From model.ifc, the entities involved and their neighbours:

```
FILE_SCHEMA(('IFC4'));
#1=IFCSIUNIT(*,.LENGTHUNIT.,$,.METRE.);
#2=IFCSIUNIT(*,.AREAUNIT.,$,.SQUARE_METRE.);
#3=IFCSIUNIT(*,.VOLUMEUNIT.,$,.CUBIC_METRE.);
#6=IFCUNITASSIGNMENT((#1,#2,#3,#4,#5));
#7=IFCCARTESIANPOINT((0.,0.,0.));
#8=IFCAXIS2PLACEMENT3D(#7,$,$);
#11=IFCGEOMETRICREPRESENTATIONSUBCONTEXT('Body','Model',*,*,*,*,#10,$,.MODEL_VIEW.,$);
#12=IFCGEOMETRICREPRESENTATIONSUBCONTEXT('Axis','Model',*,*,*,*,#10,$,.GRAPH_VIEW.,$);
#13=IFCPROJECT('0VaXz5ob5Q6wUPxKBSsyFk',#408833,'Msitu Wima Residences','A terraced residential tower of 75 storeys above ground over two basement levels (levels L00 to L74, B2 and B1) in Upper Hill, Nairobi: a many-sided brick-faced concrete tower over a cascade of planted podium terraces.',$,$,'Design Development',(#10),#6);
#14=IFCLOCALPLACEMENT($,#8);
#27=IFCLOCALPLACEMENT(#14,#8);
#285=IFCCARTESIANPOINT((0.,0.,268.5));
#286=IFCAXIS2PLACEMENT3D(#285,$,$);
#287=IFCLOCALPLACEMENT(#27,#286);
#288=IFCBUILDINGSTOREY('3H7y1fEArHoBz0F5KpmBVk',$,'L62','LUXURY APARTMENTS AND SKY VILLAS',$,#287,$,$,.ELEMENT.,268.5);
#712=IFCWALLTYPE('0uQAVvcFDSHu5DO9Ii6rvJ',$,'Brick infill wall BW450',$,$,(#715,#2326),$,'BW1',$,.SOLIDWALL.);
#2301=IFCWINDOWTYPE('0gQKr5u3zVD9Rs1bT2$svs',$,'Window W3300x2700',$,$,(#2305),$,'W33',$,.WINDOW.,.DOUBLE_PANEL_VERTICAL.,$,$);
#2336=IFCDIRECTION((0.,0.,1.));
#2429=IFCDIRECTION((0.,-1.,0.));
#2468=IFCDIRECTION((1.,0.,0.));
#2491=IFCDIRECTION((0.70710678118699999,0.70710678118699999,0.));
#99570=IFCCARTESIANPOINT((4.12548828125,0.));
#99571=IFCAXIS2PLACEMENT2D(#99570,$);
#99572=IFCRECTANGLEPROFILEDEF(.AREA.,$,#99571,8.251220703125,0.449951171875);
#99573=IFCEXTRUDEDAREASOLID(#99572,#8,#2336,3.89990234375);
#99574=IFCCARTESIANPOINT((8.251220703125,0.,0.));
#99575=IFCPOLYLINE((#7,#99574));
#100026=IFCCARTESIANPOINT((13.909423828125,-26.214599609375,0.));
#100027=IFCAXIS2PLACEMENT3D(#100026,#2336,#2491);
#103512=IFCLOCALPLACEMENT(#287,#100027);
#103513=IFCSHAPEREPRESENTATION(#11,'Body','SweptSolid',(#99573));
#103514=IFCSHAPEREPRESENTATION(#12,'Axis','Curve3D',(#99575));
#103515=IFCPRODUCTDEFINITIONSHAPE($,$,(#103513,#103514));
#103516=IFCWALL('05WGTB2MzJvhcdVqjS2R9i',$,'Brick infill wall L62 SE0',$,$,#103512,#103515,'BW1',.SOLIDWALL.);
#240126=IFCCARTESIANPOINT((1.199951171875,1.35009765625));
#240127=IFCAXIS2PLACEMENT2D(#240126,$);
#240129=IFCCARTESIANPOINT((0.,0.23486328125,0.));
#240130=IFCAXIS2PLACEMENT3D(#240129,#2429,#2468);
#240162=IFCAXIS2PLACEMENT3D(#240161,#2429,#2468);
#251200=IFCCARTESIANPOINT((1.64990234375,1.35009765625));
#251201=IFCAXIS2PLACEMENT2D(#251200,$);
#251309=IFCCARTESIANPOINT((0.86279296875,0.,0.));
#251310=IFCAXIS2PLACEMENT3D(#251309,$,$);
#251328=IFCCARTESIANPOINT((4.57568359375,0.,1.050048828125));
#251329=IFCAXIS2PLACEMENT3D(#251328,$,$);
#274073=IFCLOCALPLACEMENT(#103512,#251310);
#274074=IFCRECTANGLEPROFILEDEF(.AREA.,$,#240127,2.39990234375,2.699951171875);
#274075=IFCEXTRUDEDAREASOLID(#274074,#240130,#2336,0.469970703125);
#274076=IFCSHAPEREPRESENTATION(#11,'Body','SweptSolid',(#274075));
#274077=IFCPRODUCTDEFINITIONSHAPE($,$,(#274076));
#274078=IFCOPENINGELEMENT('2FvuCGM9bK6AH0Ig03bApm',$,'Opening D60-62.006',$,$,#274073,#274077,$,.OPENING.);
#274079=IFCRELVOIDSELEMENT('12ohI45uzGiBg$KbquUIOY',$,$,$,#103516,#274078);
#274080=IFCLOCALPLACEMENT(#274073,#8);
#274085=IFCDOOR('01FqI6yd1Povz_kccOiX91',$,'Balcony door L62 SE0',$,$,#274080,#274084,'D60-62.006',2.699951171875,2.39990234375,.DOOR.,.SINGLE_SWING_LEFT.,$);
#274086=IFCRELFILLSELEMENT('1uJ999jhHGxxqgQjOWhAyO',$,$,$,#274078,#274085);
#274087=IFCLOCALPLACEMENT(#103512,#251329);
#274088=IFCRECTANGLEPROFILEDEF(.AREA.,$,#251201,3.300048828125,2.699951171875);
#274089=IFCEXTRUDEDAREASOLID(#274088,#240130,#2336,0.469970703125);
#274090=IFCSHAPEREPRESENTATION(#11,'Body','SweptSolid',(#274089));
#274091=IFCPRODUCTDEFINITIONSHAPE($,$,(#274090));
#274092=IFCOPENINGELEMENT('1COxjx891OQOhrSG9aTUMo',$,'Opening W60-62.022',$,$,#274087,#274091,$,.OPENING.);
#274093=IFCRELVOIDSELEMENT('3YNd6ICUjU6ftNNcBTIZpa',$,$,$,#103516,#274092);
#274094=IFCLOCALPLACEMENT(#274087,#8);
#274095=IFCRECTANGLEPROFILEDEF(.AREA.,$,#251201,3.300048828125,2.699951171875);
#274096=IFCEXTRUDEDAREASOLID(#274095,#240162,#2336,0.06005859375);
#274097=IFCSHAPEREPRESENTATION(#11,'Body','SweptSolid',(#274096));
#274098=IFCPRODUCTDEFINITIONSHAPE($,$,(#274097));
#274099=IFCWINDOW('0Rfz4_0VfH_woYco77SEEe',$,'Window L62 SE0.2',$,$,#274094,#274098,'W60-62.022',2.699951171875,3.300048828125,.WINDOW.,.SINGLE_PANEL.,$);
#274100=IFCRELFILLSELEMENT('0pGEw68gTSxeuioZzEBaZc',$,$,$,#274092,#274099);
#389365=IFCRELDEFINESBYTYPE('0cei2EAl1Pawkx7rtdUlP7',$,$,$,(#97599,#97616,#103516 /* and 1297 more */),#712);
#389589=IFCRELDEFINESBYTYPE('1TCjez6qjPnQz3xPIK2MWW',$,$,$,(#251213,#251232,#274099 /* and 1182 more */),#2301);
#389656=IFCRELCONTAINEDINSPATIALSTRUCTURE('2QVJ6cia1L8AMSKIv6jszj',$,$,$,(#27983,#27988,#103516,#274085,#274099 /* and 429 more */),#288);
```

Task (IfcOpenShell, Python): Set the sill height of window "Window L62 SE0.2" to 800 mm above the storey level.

```python
import numpy as np
import ifcopenshell
import ifcopenshell.api.geometry
import ifcopenshell.geom
import ifcopenshell.util.element
import ifcopenshell.util.placement
import ifcopenshell.util.shape
import ifcopenshell.util.unit

model = ifcopenshell.open("model.ifc")
unit_scale = ifcopenshell.util.unit.calculate_unit_scale(model)

window = model.by_id(274099)
opening = window.FillsVoids[0].RelatingOpeningElement
storey = ifcopenshell.util.element.get_container(window, ifc_class="IfcBuildingStorey")
level = ifcopenshell.util.placement.get_local_placement(storey.ObjectPlacement)[2, 3]

# The opening's origin need not be at the sill, so measure its lowest point.
shape = ifcopenshell.geom.create_shape(ifcopenshell.geom.settings(), opening)
bottom = ifcopenshell.util.shape.get_shape_bottom_elevation(shape, shape.geometry) / unit_scale
dz = level + 0.8 - bottom

shift = np.array([0.0, 0.0, dz])
# The window is placed relative to its opening, so it follows when the opening moves.
matrix = ifcopenshell.util.placement.get_local_placement(opening.ObjectPlacement)
matrix[:3, 3] += shift
ifcopenshell.api.geometry.edit_object_placement(
    model, product=opening, matrix=matrix, is_si=False, should_transform_children=True
)

print(f"moved by {dz * unit_scale:+.3f} m")

model.write("model-out.ifc")
```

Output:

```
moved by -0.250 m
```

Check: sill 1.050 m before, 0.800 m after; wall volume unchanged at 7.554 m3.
